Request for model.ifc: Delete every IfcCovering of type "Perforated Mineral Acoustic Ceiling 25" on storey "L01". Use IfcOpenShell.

First a look at what the model holds.

```python
import ifcopenshell
import ifcopenshell.util.element

model = ifcopenshell.open("model.ifc")
print(model.schema)
storey = next(s for s in model.by_type("IfcBuildingStorey") if s.Name == "L01")
coverings = [e for e in ifcopenshell.util.element.get_decomposition(storey) if e.is_a("IfcCovering")]
seen = {}
for e in coverings:
    element_type = ifcopenshell.util.element.get_type(e)
    name = element_type.Name if element_type not in (None, e) else None
    seen[name] = seen.get(name, 0) + 1
for name, count in sorted(seen.items(), key=str):
    print(count, "x", name)
```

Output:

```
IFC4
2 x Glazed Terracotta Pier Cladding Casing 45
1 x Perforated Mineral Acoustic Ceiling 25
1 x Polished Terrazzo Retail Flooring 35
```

```python
import ifcopenshell
import ifcopenshell.api.root
import ifcopenshell.util.element

model = ifcopenshell.open("model.ifc")

storey = next(s for s in model.by_type("IfcBuildingStorey") if s.Name == "L01")
coverings = [e for e in ifcopenshell.util.element.get_decomposition(storey) if e.is_a("IfcCovering")]
targets = [e for e in coverings if (t := ifcopenshell.util.element.get_type(e)) not in (None, e) and t.Name == "Perforated Mineral Acoustic Ceiling 25"]

for e in targets:
    ifcopenshell.api.root.remove_product(model, product=e)
print(len(targets), "removed")

model.write("model_v2.ifc")
```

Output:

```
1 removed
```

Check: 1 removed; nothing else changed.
